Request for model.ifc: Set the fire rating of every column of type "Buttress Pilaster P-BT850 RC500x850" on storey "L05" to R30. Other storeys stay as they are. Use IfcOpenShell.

First a look at what the model holds.

```python
import ifcopenshell
import ifcopenshell.util.element

model = ifcopenshell.open("model.ifc")
print(model.schema)
storey = next(s for s in model.by_type("IfcBuildingStorey") if s.Name == "L05")
columns = [e for e in ifcopenshell.util.element.get_decomposition(storey) if e.is_a("IfcColumn")]
seen = {}
for e in columns:
    element_type = ifcopenshell.util.element.get_type(e)
    key = (element_type.Name if element_type != e and element_type else None, ifcopenshell.util.element.get_pset(e, "Pset_ColumnCommon", "FireRating"))
    seen[key] = seen.get(key, 0) + 1
for (name, value), count in sorted(seen.items(), key=str):
    print(count, "x", name, "|", value)
```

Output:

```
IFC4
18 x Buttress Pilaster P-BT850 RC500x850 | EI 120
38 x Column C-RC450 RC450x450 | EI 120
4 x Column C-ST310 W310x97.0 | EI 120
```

```python
import ifcopenshell
import ifcopenshell.api.pset
import ifcopenshell.util.element

model = ifcopenshell.open("model.ifc")

storey = next(s for s in model.by_type("IfcBuildingStorey") if s.Name == "L05")
columns = [e for e in ifcopenshell.util.element.get_decomposition(storey) if e.is_a("IfcColumn")]

count = 0
for e in columns:
    element_type = ifcopenshell.util.element.get_type(e)
    if element_type in (None, e) or element_type.Name != "Buttress Pilaster P-BT850 RC500x850":
        continue
    # add_pset returns the element's existing set when there is one.
    pset = ifcopenshell.api.pset.add_pset(model, product=e, name="Pset_ColumnCommon")
    ifcopenshell.api.pset.edit_pset(model, pset=pset, properties={"FireRating": "R30"})
    count += 1

print(count, "columns updated")

model.write("model_v2.ifc")
```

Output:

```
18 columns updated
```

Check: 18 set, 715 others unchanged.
